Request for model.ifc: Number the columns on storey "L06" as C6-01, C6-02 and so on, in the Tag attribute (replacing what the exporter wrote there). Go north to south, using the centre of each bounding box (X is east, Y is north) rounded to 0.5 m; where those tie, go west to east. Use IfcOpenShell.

First a look at what the model holds.

```python
import ifcopenshell
import ifcopenshell.util.element
import ifcopenshell.util.placement

model = ifcopenshell.open("model.ifc")
print(model.schema)
storey = next(s for s in model.by_type("IfcBuildingStorey") if s.Name == "L06")
columns = [e for e in ifcopenshell.util.element.get_decomposition(storey) if e.is_a("IfcColumn")]
for e in sorted(columns, key=lambda e: e.id()):
    origin = ifcopenshell.util.placement.get_local_placement(e.ObjectPlacement)[:3, 3]
    print(e.id(), e.Tag, e.Name, origin.round(2) + 0.0, sep=" | ")
```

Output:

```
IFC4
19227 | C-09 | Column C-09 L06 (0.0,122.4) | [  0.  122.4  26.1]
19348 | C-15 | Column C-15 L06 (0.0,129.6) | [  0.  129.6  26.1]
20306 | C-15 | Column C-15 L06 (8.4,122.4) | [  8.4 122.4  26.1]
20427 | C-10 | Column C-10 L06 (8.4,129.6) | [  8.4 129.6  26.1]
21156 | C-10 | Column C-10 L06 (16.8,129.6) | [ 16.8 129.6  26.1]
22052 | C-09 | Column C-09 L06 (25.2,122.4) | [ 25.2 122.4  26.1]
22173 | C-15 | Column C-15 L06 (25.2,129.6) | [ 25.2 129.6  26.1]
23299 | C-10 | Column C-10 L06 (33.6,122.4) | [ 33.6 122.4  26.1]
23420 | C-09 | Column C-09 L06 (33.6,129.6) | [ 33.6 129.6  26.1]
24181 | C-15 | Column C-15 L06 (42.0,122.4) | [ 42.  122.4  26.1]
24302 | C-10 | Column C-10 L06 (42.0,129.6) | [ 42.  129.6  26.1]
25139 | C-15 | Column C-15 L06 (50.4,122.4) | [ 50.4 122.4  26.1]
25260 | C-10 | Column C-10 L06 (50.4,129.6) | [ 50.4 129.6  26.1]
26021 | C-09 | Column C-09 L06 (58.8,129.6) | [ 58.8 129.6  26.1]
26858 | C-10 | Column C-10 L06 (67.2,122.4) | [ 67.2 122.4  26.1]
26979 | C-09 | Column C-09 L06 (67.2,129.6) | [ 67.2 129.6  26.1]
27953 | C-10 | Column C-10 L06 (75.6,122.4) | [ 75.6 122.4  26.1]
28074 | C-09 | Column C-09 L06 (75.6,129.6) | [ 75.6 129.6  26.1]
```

```python
import ifcopenshell
import ifcopenshell.geom
import ifcopenshell.util.element
import ifcopenshell.util.shape

model = ifcopenshell.open("model.ifc")
settings = ifcopenshell.geom.settings()
settings.set("use-world-coords", True)


def centre(element):
    shape = ifcopenshell.geom.create_shape(settings, element)
    return ifcopenshell.util.shape.get_bbox_centroid(shape.geometry)


storey = next(s for s in model.by_type("IfcBuildingStorey") if s.Name == "L06")
columns = [e for e in ifcopenshell.util.element.get_decomposition(storey) if e.is_a("IfcColumn")]

# Insertion points can sit at a corner or the storey origin, so sort by the geometry (in metres).
centres = {e: centre(e) for e in columns}
columns.sort(key=lambda e: (-round(centres[e][1] / 0.5), centres[e][0]))

for i, e in enumerate(columns, start=1):
    number = f"C6-{i:02d}"
    e.Tag = number
    print(e.id(), number)

model.write("model_updated.ifc")
```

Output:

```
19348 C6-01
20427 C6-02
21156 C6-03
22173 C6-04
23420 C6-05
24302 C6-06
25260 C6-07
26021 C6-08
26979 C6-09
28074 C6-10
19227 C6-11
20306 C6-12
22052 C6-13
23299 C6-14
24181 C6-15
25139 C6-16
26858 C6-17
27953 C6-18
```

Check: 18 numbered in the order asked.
